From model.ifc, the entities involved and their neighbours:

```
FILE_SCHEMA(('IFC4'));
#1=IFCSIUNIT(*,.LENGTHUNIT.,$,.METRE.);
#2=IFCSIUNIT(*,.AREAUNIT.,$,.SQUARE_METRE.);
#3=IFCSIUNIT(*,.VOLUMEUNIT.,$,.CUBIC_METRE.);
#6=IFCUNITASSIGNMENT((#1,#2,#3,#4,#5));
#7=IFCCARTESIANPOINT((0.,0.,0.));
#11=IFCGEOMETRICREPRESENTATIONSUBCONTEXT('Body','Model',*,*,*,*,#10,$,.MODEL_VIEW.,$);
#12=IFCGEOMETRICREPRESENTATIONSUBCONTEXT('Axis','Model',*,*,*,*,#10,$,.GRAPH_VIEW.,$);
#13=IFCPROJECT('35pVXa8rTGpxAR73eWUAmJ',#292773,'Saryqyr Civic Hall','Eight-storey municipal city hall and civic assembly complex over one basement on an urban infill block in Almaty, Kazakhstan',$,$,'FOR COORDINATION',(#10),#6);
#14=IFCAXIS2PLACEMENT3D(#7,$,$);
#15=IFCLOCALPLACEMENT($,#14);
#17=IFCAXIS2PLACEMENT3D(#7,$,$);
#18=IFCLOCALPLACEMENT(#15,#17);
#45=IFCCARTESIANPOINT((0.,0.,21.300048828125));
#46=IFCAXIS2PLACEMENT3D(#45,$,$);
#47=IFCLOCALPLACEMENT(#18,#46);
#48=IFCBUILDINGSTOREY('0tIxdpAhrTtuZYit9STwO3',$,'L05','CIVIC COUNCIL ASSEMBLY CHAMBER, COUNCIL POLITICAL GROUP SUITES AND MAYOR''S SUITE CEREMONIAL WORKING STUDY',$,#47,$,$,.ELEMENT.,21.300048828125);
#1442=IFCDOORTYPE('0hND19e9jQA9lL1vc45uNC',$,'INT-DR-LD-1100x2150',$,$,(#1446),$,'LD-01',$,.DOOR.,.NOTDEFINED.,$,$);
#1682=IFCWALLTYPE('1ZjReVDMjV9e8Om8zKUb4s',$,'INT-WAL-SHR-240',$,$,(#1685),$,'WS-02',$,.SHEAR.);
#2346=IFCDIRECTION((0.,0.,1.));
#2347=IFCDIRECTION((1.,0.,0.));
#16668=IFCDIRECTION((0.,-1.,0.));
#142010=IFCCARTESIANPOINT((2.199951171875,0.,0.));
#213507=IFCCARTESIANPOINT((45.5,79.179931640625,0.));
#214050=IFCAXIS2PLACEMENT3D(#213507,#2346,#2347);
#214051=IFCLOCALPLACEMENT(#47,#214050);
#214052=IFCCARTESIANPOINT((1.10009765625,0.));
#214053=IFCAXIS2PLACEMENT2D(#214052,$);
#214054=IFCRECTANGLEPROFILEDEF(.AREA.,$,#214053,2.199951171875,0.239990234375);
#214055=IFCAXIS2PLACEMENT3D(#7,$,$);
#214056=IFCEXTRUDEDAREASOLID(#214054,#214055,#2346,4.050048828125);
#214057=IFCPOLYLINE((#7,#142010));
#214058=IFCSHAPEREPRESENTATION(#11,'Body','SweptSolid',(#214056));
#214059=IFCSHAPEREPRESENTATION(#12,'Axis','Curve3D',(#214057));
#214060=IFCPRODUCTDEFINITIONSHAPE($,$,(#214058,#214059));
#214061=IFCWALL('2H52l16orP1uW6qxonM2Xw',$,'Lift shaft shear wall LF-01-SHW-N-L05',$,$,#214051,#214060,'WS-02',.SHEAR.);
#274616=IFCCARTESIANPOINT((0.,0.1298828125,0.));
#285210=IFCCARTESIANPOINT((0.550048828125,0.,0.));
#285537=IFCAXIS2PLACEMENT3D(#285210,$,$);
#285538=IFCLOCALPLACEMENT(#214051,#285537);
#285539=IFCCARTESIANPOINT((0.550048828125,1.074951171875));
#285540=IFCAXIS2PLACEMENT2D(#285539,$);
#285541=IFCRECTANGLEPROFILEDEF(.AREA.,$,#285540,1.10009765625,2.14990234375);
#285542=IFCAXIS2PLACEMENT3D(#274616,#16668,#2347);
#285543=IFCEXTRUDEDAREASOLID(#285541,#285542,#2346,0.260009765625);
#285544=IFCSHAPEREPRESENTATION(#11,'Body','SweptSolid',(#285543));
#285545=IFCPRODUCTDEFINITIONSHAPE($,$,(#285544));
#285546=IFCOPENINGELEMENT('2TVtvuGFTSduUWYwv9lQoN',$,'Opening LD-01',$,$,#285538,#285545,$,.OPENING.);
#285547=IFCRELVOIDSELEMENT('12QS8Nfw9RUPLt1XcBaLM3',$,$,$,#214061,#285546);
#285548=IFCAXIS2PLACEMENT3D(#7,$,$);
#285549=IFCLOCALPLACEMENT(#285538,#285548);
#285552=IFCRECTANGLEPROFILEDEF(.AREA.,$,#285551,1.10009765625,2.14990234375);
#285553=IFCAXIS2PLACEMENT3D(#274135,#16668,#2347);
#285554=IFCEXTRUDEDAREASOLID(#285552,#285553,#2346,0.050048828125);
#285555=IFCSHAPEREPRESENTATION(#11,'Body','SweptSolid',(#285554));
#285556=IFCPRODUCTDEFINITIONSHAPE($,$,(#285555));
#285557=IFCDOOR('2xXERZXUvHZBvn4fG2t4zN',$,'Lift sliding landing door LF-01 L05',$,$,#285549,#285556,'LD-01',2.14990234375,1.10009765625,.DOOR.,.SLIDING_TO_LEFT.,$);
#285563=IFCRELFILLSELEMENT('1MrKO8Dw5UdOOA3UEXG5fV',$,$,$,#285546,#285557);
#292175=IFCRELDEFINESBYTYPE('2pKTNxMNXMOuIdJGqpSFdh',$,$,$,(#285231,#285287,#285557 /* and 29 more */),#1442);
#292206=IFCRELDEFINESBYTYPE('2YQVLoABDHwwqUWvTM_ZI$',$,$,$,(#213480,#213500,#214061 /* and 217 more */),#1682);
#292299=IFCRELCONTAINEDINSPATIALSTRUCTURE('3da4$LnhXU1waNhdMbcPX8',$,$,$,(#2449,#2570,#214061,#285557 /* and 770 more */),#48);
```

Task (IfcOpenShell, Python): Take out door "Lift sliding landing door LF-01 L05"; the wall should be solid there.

```python
import ifcopenshell
import ifcopenshell.api.feature
import ifcopenshell.api.root
import ifcopenshell.geom
import ifcopenshell.util.shape

model = ifcopenshell.open("model.ifc")
settings = ifcopenshell.geom.settings()


def volume(element):
    """Net volume in cubic metres, openings subtracted."""
    shape = ifcopenshell.geom.create_shape(settings, element)
    return ifcopenshell.util.shape.get_volume(shape.geometry)


door = model.by_guid("2xXERZXUvHZBvn4fG2t4zN")
opening = door.FillsVoids[0].RelatingOpeningElement
wall = opening.VoidsElements[0].RelatingBuildingElement
before = volume(wall)

ifcopenshell.api.root.remove_product(model, product=door)
ifcopenshell.api.feature.remove_feature(model, feature=opening)

after = volume(wall)

print(f"wall volume {before:.3f} -> {after:.3f} m3")

model.write("model_updated.ifc")
```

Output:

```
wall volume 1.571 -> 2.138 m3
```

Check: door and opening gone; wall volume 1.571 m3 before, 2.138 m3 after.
